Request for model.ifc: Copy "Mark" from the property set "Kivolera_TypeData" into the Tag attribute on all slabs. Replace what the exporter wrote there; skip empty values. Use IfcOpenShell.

First a look at what the model holds.

```python
import ifcopenshell
import ifcopenshell.util.element

model = ifcopenshell.open("model.ifc")
print(model.schema)
slabs = model.by_type("IfcSlab")
print(len(slabs), "slabs")
for e in slabs[:8]:
    source = ifcopenshell.util.element.get_pset(e, "Kivolera_TypeData", "Mark")
    target = e.Tag
    print(e.id(), repr(source), repr(target), sep=" | ")
```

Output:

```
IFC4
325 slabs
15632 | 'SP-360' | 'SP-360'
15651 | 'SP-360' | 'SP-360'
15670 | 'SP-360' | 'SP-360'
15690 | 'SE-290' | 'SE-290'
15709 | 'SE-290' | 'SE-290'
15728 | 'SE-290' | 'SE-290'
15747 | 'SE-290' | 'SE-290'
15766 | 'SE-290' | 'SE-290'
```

```python
import ifcopenshell
import ifcopenshell.util.element

model = ifcopenshell.open("model.ifc")

count = 0
for e in model.by_type("IfcSlab"):
    value = ifcopenshell.util.element.get_pset(e, "Kivolera_TypeData", "Mark")
    current = e.Tag
    if not value or not value.strip() or current == value:
        continue
    e.Tag = value
    count += 1

print(count, "slabs updated")

model.write("model_updated.ifc")
```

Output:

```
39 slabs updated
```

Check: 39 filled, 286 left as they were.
